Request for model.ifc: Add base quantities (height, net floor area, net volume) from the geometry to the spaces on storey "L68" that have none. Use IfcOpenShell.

First a look at what the model holds.

```python
import ifcopenshell
import ifcopenshell.util.element
import ifcopenshell.util.unit

model = ifcopenshell.open("model.ifc")
print(model.schema)
for unit_type in ("LENGTHUNIT", "AREAUNIT", "VOLUMEUNIT"):
    print(unit_type, ifcopenshell.util.unit.calculate_unit_scale(model, unit_type))
storey = next(s for s in model.by_type("IfcBuildingStorey") if s.Name == "L68")
spaces = [e for e in ifcopenshell.util.element.get_decomposition(storey) if e.is_a("IfcSpace")]
for e in sorted(spaces, key=lambda e: e.id()):
    print(e.id(), e.is_a(), e.Name, list(ifcopenshell.util.element.get_psets(e, qtos_only=True)), sep=" | ")
```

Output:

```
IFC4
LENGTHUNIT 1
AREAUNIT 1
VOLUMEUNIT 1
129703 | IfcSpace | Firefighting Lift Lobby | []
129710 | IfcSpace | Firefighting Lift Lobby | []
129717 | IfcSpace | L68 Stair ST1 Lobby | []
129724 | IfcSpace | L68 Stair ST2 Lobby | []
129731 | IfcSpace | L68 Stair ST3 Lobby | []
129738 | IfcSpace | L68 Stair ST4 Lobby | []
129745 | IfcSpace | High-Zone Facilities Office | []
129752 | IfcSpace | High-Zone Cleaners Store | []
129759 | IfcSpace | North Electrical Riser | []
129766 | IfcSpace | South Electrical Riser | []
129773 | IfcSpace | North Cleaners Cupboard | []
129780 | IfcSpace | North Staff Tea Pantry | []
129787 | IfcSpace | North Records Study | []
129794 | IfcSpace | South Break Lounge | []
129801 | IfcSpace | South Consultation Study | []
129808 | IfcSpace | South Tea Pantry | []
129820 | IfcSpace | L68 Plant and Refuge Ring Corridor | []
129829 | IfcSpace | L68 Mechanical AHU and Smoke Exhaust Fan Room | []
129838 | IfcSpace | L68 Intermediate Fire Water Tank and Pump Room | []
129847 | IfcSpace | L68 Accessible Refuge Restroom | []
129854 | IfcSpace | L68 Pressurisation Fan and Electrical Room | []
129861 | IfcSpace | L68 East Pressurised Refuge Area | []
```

```python
import ifcopenshell
import ifcopenshell.api.pset
import ifcopenshell.geom
import ifcopenshell.util.element
import ifcopenshell.util.shape
import ifcopenshell.util.unit

model = ifcopenshell.open("model.ifc")
unit_scale = ifcopenshell.util.unit.calculate_unit_scale(model)
area_scale = ifcopenshell.util.unit.calculate_unit_scale(model, "AREAUNIT")
volume_scale = ifcopenshell.util.unit.calculate_unit_scale(model, "VOLUMEUNIT")
settings = ifcopenshell.geom.settings()

storey = next(s for s in model.by_type("IfcBuildingStorey") if s.Name == "L68")
spaces = [e for e in ifcopenshell.util.element.get_decomposition(storey) if e.is_a("IfcSpace")]

for e in sorted(spaces, key=lambda e: e.id()):
    if ifcopenshell.util.element.get_psets(e, qtos_only=True, should_inherit=False):
        continue
    # Geometry comes back in metres, in the element's own axes.
    shape = ifcopenshell.geom.create_shape(settings, e)
    values = {
        "Height": ifcopenshell.util.shape.get_z(shape.geometry) / unit_scale,
        "NetFloorArea": ifcopenshell.util.shape.get_footprint_area(shape.geometry) / area_scale,
        "NetVolume": ifcopenshell.util.shape.get_volume(shape.geometry) / volume_scale,
    }
    qto = ifcopenshell.api.pset.add_qto(model, product=e, name="Qto_SpaceBaseQuantities")
    ifcopenshell.api.pset.edit_qto(model, qto=qto, properties=values)
    print(e.id(), {k: round(v, 3) for k, v in values.items()})

model.write("model_v2.ifc")
```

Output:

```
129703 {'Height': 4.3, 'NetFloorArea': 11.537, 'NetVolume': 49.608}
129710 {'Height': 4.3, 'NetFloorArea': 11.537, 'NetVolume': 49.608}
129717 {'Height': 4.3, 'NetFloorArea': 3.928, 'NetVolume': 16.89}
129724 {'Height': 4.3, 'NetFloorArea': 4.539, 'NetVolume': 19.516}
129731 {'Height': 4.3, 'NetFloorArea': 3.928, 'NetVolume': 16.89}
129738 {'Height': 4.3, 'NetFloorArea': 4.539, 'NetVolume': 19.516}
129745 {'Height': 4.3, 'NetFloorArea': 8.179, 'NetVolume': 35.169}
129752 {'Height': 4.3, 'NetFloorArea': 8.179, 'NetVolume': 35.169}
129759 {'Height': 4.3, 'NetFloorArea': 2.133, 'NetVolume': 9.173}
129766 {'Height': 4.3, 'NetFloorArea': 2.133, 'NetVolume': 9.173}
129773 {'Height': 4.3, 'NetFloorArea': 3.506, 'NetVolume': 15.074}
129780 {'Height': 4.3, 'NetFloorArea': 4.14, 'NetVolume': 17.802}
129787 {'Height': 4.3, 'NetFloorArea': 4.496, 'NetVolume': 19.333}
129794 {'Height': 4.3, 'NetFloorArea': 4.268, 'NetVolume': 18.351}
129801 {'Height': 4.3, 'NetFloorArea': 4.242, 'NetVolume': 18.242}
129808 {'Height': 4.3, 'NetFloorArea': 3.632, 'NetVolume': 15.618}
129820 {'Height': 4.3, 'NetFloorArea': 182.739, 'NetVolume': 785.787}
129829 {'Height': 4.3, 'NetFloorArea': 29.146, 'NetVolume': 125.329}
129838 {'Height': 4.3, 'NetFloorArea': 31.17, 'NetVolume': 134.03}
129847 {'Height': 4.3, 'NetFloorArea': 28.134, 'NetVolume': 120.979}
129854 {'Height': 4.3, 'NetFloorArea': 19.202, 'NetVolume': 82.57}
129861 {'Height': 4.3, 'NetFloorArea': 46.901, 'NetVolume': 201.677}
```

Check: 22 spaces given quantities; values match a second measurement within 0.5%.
